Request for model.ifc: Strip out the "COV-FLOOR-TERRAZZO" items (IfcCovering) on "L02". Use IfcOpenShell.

First a look at what the model holds.

```python
import ifcopenshell
import ifcopenshell.util.element

model = ifcopenshell.open("model.ifc")
print(model.schema)
storey = next(s for s in model.by_type("IfcBuildingStorey") if s.Name == "L02")
coverings = [e for e in ifcopenshell.util.element.get_decomposition(storey) if e.is_a("IfcCovering")]
seen = {}
for e in coverings:
    element_type = ifcopenshell.util.element.get_type(e)
    name = element_type.Name if element_type not in (None, e) else None
    seen[name] = seen.get(name, 0) + 1
for name, count in sorted(seen.items(), key=str):
    print(count, "x", name)
```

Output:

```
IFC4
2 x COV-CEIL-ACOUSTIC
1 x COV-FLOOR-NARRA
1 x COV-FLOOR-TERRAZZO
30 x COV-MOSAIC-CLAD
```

```python
import ifcopenshell
import ifcopenshell.api.root
import ifcopenshell.util.element

model = ifcopenshell.open("model.ifc")

storey = next(s for s in model.by_type("IfcBuildingStorey") if s.Name == "L02")
coverings = [e for e in ifcopenshell.util.element.get_decomposition(storey) if e.is_a("IfcCovering")]
targets = [e for e in coverings if (t := ifcopenshell.util.element.get_type(e)) not in (None, e) and t.Name == "COV-FLOOR-TERRAZZO"]

for e in targets:
    ifcopenshell.api.root.remove_product(model, product=e)
print(len(targets), "removed")

model.write("model_rev.ifc")
```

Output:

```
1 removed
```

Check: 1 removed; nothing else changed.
